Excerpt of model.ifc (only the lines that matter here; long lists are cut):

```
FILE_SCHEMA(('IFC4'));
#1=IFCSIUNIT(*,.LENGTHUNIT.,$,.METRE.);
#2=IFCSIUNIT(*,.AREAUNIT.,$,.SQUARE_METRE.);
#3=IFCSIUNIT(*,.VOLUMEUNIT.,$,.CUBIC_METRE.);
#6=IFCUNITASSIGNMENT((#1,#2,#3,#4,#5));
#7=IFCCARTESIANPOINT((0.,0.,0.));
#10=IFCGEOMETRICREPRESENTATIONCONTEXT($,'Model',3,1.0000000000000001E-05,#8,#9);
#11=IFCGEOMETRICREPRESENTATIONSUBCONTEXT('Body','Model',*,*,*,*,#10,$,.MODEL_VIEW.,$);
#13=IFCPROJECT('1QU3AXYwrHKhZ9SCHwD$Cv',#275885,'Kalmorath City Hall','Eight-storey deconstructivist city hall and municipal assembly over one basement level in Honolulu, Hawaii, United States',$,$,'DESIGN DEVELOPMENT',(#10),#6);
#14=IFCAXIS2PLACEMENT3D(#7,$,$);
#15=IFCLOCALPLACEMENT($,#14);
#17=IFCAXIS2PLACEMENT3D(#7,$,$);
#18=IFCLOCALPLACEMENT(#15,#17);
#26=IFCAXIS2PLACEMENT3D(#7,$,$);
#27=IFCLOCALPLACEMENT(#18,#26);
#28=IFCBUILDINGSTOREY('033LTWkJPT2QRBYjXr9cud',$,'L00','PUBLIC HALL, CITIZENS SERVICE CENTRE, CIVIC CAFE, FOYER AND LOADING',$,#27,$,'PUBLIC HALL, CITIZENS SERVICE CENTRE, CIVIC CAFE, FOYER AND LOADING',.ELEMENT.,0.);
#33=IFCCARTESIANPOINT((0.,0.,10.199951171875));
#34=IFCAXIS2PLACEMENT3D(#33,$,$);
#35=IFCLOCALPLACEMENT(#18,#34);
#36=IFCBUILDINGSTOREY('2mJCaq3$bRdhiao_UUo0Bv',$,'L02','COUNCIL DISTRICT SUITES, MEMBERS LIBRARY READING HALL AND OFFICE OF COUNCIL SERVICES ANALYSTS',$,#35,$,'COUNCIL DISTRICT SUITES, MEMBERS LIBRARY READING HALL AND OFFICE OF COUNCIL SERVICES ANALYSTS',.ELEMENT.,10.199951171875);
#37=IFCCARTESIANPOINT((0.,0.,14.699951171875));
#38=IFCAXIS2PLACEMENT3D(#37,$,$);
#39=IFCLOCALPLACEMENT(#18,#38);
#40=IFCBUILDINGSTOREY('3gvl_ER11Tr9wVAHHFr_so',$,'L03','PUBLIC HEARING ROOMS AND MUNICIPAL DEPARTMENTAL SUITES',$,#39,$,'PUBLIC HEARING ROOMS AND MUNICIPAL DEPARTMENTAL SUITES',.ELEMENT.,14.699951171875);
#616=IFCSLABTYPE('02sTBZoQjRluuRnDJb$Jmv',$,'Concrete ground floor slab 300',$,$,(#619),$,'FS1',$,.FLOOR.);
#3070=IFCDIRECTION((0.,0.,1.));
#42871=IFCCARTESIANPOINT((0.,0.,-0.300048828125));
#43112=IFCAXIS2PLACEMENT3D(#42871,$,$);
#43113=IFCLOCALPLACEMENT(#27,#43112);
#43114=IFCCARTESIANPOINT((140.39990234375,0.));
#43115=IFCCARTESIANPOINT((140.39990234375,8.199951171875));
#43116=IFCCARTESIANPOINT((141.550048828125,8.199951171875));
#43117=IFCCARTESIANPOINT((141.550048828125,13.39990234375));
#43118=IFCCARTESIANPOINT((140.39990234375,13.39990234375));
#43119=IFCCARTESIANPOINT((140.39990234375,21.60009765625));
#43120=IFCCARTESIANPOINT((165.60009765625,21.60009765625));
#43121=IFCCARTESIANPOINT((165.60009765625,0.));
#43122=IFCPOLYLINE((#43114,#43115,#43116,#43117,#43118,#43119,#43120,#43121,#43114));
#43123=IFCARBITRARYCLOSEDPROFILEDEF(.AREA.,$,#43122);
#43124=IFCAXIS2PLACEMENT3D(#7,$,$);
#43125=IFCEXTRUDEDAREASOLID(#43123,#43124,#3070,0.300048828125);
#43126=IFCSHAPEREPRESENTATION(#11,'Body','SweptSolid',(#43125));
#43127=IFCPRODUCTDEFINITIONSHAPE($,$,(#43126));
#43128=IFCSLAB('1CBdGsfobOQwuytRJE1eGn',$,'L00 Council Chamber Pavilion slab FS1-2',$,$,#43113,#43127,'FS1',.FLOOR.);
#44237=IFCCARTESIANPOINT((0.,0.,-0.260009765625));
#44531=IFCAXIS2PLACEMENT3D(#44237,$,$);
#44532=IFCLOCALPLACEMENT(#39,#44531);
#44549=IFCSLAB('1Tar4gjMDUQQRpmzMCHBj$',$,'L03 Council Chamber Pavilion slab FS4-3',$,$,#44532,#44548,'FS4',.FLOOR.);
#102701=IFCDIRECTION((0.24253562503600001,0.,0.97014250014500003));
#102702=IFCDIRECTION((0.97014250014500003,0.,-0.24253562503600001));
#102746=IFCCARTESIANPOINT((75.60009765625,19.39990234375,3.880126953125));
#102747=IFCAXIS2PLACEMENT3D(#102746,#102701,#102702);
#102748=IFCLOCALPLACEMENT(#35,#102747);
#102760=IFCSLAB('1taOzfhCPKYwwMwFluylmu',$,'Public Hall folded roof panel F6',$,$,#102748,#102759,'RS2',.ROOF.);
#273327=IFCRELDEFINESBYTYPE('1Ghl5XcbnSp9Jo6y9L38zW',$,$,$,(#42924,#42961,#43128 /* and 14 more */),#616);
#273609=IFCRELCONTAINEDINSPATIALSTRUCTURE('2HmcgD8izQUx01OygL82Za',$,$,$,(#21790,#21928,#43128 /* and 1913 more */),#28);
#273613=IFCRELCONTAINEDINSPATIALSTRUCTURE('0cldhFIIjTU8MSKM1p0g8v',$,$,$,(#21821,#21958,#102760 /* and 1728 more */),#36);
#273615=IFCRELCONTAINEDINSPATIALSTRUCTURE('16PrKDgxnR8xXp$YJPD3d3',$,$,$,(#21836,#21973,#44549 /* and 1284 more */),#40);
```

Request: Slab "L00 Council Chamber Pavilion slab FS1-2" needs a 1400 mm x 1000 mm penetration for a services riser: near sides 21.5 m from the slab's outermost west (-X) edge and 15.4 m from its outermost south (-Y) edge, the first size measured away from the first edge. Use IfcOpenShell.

```python
import numpy as np
import ifcopenshell
import ifcopenshell.api.feature
import ifcopenshell.api.geometry
import ifcopenshell.api.root
import ifcopenshell.geom
import ifcopenshell.util.placement
import ifcopenshell.util.representation
import ifcopenshell.util.shape
import ifcopenshell.util.unit

model = ifcopenshell.open("model.ifc")
unit_scale = ifcopenshell.util.unit.calculate_unit_scale(model)
settings = ifcopenshell.geom.settings()


def volume(element):
    """Net volume in cubic metres, openings subtracted."""
    shape = ifcopenshell.geom.create_shape(settings, element)
    return ifcopenshell.util.shape.get_volume(shape.geometry)


slab = model.by_guid("1CBdGsfobOQwuytRJE1eGn")
before = volume(slab)

# Extent in the slab's own axes, in metres. The edges named are its -X and -Y sides.
slab_shape = ifcopenshell.geom.create_shape(settings, slab)
vertices = ifcopenshell.util.shape.get_vertices(slab_shape.geometry)
x_min, y_min, bottom = vertices.min(axis=0)
top = vertices[:, 2].max()

opening = ifcopenshell.api.root.create_entity(model, ifc_class="IfcOpeningElement", name="Services riser opening", predefined_type="OPENING")
context = ifcopenshell.util.representation.get_context(model, "Model", "Body", "MODEL_VIEW")
width, depth = 1.4, 1
outline = [(0.0, 0.0), (width, 0.0), (width, depth), (0.0, depth), (0.0, 0.0)]
# Overshoot both faces by 50 mm so the cut is clean.
shape = ifcopenshell.api.geometry.add_slab_representation(
    model, context=context, depth=top - bottom + 0.1, polyline=outline
)
ifcopenshell.api.geometry.assign_representation(model, product=opening, representation=shape)

matrix = ifcopenshell.util.placement.get_local_placement(slab.ObjectPlacement)
matrix[:, 3] = matrix @ np.append(np.array([x_min + 21.5, y_min + 15.4, bottom - 0.05]) / unit_scale, 1.0)
ifcopenshell.api.geometry.edit_object_placement(model, product=opening, matrix=matrix, is_si=False)
ifcopenshell.api.feature.add_feature(model, feature=opening, element=slab)

after = volume(slab)

print(f"slab volume {before:.3f} -> {after:.3f} m3")

model.write("model_rev.ifc")
```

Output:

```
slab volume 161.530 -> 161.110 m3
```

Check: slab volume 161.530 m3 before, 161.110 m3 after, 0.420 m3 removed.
